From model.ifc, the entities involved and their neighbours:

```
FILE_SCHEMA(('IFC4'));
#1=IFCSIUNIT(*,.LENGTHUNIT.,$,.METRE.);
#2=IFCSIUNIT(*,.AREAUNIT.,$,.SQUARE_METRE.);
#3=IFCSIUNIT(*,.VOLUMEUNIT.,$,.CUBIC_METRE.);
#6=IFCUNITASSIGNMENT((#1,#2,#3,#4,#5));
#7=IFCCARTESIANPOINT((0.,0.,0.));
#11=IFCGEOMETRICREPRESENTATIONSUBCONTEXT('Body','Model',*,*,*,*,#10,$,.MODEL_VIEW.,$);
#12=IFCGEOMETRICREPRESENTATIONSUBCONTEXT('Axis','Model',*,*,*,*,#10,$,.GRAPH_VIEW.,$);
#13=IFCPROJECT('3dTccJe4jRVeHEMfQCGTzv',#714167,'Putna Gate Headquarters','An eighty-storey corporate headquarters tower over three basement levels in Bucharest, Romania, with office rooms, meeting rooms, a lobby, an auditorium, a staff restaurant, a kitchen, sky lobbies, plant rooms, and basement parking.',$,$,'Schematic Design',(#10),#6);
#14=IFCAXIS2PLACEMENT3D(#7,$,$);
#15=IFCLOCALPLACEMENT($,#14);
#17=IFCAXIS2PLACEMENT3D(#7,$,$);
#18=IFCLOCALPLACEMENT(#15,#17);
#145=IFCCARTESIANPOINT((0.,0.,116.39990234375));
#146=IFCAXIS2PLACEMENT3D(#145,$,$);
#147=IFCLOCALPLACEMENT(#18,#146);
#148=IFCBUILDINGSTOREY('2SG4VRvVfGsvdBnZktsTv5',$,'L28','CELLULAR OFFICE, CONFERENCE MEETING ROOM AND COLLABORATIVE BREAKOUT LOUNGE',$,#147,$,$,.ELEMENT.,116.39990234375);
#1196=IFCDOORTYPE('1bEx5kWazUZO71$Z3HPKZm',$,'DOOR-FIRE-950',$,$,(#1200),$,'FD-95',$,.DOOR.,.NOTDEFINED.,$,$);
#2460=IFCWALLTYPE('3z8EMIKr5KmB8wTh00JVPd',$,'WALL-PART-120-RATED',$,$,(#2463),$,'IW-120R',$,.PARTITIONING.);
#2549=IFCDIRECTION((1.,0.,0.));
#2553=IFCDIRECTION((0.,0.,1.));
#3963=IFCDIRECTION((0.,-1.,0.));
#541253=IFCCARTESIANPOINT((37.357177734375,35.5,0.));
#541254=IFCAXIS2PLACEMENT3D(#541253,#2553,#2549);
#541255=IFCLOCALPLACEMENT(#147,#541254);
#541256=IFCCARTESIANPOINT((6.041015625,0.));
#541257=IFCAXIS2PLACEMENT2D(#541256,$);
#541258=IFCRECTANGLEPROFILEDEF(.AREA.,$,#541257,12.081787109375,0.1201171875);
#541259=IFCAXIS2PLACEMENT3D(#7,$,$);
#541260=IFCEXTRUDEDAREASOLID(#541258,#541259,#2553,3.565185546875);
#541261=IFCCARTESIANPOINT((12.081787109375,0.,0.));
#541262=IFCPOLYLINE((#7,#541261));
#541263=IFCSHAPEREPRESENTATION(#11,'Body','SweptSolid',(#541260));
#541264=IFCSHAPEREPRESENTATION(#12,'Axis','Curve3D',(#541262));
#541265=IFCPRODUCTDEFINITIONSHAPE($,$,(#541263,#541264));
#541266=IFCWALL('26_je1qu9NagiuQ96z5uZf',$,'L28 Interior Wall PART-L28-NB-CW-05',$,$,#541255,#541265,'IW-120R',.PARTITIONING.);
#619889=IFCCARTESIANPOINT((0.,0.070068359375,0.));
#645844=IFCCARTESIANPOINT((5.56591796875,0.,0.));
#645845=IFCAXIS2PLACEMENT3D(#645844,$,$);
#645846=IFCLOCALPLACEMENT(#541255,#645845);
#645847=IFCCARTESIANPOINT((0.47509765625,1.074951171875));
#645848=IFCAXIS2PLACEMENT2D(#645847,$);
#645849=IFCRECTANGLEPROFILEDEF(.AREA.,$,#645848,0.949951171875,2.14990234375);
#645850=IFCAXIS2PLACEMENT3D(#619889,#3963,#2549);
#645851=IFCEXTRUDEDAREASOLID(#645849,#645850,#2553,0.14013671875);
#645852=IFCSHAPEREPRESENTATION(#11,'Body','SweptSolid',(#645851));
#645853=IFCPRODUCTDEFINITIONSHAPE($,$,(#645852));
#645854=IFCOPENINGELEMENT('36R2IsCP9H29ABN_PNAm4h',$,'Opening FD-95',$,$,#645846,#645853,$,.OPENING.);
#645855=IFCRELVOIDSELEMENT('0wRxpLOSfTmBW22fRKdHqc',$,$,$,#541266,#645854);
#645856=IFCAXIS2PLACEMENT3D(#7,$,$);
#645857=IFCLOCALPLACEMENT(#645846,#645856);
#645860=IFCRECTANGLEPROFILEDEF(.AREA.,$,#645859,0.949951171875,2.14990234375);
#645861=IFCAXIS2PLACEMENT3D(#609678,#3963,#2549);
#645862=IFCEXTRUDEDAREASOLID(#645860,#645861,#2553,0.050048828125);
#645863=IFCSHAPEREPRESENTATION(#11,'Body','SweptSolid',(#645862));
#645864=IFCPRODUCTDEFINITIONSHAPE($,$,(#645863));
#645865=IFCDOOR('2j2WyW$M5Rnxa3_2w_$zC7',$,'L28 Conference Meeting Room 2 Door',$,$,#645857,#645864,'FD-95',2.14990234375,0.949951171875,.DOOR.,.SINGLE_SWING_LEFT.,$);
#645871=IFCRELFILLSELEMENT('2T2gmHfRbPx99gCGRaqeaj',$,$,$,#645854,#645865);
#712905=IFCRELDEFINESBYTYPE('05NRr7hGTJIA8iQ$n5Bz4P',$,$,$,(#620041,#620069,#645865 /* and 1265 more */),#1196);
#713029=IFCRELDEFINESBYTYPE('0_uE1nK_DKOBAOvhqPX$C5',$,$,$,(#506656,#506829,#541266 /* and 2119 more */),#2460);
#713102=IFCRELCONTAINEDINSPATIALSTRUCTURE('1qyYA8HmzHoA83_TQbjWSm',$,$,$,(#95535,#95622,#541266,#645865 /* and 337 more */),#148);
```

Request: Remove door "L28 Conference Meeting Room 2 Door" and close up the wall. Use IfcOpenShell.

```python
import ifcopenshell
import ifcopenshell.api.feature
import ifcopenshell.api.root
import ifcopenshell.geom
import ifcopenshell.util.shape

model = ifcopenshell.open("model.ifc")
settings = ifcopenshell.geom.settings()


def volume(element):
    """Net volume in cubic metres, openings subtracted."""
    shape = ifcopenshell.geom.create_shape(settings, element)
    return ifcopenshell.util.shape.get_volume(shape.geometry)


door = model.by_guid("2j2WyW$M5Rnxa3_2w_$zC7")
opening = door.FillsVoids[0].RelatingOpeningElement
wall = opening.VoidsElements[0].RelatingBuildingElement
before = volume(wall)

ifcopenshell.api.root.remove_product(model, product=door)
ifcopenshell.api.feature.remove_feature(model, feature=opening)

after = volume(wall)

print(f"wall volume {before:.3f} -> {after:.3f} m3")

model.write("model_rev.ifc")
```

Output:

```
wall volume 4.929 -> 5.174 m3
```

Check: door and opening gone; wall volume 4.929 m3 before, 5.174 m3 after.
